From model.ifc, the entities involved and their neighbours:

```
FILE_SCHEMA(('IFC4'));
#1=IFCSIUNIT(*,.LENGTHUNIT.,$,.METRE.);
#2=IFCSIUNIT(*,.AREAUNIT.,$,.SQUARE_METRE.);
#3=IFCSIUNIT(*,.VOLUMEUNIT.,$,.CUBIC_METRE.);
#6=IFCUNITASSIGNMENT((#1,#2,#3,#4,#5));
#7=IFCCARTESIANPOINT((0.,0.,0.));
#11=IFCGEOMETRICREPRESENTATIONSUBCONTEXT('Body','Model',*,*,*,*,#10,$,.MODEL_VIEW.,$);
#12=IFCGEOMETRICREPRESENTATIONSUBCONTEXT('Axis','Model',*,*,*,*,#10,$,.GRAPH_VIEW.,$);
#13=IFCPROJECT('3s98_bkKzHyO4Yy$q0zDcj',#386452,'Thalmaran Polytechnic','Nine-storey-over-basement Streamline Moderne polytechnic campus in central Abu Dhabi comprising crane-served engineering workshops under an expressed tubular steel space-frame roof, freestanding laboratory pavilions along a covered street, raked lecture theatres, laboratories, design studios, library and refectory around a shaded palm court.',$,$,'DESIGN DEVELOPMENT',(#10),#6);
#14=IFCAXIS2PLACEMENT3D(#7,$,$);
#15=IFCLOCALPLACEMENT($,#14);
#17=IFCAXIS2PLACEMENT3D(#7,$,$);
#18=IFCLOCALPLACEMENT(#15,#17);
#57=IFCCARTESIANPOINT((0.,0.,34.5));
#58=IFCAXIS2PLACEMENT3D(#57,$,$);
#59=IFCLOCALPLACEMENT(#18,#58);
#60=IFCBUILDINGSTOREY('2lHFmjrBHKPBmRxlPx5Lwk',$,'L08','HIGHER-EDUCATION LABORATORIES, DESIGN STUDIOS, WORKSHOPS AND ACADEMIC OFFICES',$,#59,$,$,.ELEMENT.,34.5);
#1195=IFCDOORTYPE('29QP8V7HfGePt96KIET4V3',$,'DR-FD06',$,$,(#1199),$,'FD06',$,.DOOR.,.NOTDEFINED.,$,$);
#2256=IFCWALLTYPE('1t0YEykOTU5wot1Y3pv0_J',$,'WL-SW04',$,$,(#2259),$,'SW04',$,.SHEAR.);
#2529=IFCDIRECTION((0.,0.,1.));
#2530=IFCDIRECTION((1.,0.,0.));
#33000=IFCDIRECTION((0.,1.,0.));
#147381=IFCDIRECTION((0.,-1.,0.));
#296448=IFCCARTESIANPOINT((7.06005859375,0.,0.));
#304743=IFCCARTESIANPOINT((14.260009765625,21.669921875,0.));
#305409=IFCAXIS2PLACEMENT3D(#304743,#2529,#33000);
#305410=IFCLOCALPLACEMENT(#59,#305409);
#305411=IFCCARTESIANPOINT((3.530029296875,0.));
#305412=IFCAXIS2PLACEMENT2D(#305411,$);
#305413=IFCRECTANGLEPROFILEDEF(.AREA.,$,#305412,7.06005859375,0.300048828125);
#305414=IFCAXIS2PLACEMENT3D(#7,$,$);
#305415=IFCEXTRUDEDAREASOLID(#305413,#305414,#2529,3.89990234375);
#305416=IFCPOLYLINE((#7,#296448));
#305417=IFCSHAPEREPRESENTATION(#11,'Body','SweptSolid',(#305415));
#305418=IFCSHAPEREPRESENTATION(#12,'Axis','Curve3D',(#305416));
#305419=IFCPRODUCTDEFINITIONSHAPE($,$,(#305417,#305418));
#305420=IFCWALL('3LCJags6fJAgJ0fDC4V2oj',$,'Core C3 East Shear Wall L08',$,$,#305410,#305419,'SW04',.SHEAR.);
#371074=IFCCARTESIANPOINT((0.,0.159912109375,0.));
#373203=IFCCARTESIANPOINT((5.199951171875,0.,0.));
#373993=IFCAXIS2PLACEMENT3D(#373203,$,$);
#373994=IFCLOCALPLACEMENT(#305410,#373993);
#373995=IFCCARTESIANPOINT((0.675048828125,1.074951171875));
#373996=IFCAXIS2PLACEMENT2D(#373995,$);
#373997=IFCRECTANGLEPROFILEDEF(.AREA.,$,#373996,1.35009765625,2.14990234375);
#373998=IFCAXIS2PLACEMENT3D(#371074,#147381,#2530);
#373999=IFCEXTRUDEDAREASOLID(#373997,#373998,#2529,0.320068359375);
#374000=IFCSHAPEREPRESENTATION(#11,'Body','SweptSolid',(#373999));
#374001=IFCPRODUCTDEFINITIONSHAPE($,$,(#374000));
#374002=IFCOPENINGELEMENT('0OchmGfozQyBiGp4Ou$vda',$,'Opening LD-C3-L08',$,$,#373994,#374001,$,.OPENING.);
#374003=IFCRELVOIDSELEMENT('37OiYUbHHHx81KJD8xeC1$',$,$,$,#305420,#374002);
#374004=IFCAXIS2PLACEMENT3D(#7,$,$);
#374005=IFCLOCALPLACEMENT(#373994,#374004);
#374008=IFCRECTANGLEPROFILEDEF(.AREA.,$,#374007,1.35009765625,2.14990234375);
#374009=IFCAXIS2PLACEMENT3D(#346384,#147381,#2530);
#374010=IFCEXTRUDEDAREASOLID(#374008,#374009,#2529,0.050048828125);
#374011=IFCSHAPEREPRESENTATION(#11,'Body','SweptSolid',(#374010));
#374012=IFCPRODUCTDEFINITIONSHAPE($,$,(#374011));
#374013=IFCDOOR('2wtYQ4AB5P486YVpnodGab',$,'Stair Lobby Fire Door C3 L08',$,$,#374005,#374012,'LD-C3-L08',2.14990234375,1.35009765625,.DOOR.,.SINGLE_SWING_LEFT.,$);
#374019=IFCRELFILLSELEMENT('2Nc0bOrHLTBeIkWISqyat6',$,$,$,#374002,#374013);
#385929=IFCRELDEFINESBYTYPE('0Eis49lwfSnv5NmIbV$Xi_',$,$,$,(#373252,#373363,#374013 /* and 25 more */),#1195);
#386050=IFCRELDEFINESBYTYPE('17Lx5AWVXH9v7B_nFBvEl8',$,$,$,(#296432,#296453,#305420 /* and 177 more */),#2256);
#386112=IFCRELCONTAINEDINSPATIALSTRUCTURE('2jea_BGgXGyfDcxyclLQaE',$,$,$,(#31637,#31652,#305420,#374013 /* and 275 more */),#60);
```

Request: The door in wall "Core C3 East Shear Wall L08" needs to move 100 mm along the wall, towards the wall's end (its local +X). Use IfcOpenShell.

```python
import ifcopenshell
import ifcopenshell.api.geometry
import ifcopenshell.util.placement
import ifcopenshell.util.unit

model = ifcopenshell.open("model.ifc")
unit_scale = ifcopenshell.util.unit.calculate_unit_scale(model)

door = model.by_id(374013)
opening = door.FillsVoids[0].RelatingOpeningElement
wall = opening.VoidsElements[0].RelatingBuildingElement

wall_matrix = ifcopenshell.util.placement.get_local_placement(wall.ObjectPlacement)
shift = wall_matrix[:3, 0] * 0.1 / unit_scale
before = ifcopenshell.util.placement.get_local_placement(door.ObjectPlacement)[:3, 3].copy()

# The door is placed relative to its opening, so it follows when the opening moves.
matrix = ifcopenshell.util.placement.get_local_placement(opening.ObjectPlacement)
matrix[:3, 3] += shift
ifcopenshell.api.geometry.edit_object_placement(
    model, product=opening, matrix=matrix, is_si=False, should_transform_children=True
)

after = ifcopenshell.util.placement.get_local_placement(door.ObjectPlacement)[:3, 3]
print("door moved by", (after - before).round(3) + 0.0)

model.write("model_rev.ifc")
```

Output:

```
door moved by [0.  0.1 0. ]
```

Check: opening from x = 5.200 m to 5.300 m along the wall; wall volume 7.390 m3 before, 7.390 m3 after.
